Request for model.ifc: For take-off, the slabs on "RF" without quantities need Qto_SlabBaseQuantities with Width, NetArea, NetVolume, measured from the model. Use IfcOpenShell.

First a look at what the model holds.

```python
import ifcopenshell
import ifcopenshell.util.element
import ifcopenshell.util.unit

model = ifcopenshell.open("model.ifc")
print(model.schema)
for unit_type in ("LENGTHUNIT", "AREAUNIT", "VOLUMEUNIT"):
    print(unit_type, ifcopenshell.util.unit.calculate_unit_scale(model, unit_type))
storey = next(s for s in model.by_type("IfcBuildingStorey") if s.Name == "RF")
slabs = [e for e in ifcopenshell.util.element.get_decomposition(storey) if e.is_a("IfcSlab")]
for e in sorted(slabs, key=lambda e: e.id()):
    print(e.id(), e.is_a(), e.Name, list(ifcopenshell.util.element.get_psets(e, qtos_only=True)), sep=" | ")
```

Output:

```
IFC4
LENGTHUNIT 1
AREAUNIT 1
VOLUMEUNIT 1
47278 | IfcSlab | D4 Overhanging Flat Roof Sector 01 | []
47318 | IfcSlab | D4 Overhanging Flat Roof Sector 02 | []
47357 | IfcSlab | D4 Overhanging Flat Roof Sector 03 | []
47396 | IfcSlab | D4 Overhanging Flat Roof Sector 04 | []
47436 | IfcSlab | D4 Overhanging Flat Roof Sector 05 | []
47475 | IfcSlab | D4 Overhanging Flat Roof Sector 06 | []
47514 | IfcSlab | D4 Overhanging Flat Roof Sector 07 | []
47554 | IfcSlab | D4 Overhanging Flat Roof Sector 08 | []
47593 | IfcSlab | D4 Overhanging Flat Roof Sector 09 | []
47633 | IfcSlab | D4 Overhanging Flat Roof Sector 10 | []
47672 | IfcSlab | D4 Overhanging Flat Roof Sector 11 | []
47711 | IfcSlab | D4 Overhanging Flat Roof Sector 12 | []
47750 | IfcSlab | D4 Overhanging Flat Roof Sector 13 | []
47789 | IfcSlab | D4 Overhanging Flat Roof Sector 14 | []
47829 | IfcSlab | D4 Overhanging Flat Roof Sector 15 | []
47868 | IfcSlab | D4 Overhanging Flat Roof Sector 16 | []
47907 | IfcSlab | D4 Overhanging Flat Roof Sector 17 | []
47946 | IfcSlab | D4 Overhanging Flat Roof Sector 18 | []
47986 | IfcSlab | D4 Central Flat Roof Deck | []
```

```python
import ifcopenshell
import ifcopenshell.api.pset
import ifcopenshell.geom
import ifcopenshell.util.element
import ifcopenshell.util.shape
import ifcopenshell.util.unit

model = ifcopenshell.open("model.ifc")
unit_scale = ifcopenshell.util.unit.calculate_unit_scale(model)
area_scale = ifcopenshell.util.unit.calculate_unit_scale(model, "AREAUNIT")
volume_scale = ifcopenshell.util.unit.calculate_unit_scale(model, "VOLUMEUNIT")
settings = ifcopenshell.geom.settings()

storey = next(s for s in model.by_type("IfcBuildingStorey") if s.Name == "RF")
slabs = [e for e in ifcopenshell.util.element.get_decomposition(storey) if e.is_a("IfcSlab")]

for e in sorted(slabs, key=lambda e: e.id()):
    if ifcopenshell.util.element.get_psets(e, qtos_only=True, should_inherit=False):
        continue
    # Geometry comes back in metres, in the element's own axes.
    shape = ifcopenshell.geom.create_shape(settings, e)
    values = {
        "Width": ifcopenshell.util.shape.get_z(shape.geometry) / unit_scale,
        "NetArea": ifcopenshell.util.shape.get_footprint_area(shape.geometry) / area_scale,
        "NetVolume": ifcopenshell.util.shape.get_volume(shape.geometry) / volume_scale,
    }
    qto = ifcopenshell.api.pset.add_qto(model, product=e, name="Qto_SlabBaseQuantities")
    ifcopenshell.api.pset.edit_qto(model, qto=qto, properties=values)
    print(e.id(), {k: round(v, 3) for k, v in values.items()})

model.write("model_v2.ifc")
```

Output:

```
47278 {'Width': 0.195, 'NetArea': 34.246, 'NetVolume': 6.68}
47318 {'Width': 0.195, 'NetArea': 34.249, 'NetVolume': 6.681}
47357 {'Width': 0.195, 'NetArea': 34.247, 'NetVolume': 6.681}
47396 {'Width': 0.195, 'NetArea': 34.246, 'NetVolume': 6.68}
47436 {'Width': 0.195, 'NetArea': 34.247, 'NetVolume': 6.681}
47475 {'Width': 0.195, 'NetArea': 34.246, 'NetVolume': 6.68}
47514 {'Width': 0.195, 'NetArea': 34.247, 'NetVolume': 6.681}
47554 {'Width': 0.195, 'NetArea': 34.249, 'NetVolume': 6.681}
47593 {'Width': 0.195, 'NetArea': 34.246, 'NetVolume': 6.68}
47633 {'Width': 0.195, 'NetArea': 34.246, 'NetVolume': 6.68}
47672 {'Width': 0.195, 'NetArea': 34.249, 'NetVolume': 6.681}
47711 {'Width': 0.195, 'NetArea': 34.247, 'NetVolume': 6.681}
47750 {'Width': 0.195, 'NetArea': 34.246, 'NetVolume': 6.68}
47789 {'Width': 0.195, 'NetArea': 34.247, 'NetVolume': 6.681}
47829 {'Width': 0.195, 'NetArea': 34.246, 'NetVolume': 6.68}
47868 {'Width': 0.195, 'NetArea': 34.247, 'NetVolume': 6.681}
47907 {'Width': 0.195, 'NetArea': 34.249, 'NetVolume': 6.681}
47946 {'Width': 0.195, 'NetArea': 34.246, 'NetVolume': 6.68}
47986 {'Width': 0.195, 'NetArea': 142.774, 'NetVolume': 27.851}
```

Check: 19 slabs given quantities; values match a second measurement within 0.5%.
